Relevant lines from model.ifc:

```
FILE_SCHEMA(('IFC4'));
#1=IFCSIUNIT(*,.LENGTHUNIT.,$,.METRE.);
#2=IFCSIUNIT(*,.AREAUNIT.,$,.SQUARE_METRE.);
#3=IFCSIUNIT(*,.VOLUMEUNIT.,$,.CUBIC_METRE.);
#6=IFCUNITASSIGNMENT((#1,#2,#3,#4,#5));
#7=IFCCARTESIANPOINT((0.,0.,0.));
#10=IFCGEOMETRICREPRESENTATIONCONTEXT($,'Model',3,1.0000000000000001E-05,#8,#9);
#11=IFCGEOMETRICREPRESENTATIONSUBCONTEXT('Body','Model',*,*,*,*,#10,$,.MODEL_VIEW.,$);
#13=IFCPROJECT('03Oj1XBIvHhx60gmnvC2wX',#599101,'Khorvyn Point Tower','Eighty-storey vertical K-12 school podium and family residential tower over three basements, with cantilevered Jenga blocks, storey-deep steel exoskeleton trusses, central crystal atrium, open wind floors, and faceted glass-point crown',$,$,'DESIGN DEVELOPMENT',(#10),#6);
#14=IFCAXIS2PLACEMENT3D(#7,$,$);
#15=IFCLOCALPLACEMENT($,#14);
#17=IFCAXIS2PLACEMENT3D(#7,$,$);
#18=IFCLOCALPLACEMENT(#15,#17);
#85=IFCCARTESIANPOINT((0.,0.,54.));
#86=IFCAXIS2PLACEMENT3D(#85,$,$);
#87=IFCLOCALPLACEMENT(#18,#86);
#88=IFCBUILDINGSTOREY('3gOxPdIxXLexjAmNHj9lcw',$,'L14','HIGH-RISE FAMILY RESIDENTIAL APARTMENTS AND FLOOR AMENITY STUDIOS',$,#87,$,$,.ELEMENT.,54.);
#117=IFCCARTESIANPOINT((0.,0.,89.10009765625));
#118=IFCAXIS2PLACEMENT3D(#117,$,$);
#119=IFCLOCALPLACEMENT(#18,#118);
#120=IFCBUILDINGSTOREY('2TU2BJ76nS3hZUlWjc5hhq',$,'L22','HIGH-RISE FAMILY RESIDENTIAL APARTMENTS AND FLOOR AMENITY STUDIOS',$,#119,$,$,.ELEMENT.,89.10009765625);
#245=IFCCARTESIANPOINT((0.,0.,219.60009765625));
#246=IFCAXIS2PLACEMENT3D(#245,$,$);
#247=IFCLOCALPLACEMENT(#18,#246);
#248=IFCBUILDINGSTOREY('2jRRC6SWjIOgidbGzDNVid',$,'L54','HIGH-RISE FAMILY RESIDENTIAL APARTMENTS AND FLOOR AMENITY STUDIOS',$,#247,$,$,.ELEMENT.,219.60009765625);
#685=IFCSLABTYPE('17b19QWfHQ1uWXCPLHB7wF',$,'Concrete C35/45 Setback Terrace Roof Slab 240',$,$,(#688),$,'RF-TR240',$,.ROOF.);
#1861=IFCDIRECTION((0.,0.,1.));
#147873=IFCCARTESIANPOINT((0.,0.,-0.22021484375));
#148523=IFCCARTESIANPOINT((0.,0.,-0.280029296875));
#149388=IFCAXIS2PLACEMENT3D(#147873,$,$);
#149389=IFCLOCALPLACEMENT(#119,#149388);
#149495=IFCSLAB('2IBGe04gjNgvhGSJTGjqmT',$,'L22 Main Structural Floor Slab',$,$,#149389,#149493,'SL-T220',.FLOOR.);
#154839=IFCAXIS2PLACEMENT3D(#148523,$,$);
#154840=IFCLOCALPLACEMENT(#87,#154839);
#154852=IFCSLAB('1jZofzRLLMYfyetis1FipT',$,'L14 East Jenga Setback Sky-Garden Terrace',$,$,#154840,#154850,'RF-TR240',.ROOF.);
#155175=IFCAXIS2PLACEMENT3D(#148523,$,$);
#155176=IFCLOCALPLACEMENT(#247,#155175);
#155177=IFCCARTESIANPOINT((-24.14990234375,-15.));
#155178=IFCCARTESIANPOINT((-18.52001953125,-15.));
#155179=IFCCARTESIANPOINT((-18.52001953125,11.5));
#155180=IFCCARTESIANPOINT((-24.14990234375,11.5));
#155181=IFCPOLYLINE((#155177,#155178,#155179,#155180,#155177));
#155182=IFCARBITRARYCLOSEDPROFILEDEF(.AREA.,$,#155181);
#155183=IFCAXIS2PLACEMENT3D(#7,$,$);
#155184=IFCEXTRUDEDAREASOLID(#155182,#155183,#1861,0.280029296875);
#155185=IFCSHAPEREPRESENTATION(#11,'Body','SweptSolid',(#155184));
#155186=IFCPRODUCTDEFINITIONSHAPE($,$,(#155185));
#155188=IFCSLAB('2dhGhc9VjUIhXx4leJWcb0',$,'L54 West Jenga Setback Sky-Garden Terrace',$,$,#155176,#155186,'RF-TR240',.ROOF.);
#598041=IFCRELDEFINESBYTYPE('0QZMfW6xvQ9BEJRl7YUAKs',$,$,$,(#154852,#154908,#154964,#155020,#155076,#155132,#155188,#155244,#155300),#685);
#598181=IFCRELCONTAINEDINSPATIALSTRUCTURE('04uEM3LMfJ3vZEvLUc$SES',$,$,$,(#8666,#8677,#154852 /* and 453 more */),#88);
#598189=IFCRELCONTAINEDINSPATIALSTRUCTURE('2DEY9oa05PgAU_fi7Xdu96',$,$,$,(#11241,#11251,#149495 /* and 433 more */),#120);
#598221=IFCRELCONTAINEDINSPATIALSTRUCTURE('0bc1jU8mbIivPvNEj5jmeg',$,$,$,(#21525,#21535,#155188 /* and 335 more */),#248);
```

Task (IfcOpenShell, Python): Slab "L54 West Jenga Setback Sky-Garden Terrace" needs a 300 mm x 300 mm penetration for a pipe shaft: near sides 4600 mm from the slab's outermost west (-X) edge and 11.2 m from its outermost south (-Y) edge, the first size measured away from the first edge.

```python
import numpy as np
import ifcopenshell
import ifcopenshell.api.feature
import ifcopenshell.api.geometry
import ifcopenshell.api.root
import ifcopenshell.geom
import ifcopenshell.util.placement
import ifcopenshell.util.representation
import ifcopenshell.util.shape
import ifcopenshell.util.unit

model = ifcopenshell.open("model.ifc")
unit_scale = ifcopenshell.util.unit.calculate_unit_scale(model)
settings = ifcopenshell.geom.settings()


def volume(element):
    """Net volume in cubic metres, openings subtracted."""
    shape = ifcopenshell.geom.create_shape(settings, element)
    return ifcopenshell.util.shape.get_volume(shape.geometry)


slab = model.by_guid("2dhGhc9VjUIhXx4leJWcb0")
before = volume(slab)

# Extent in the slab's own axes, in metres. The edges named are its -X and -Y sides.
slab_shape = ifcopenshell.geom.create_shape(settings, slab)
vertices = ifcopenshell.util.shape.get_vertices(slab_shape.geometry)
x_min, y_min, bottom = vertices.min(axis=0)
top = vertices[:, 2].max()

opening = ifcopenshell.api.root.create_entity(model, ifc_class="IfcOpeningElement", name="Pipe shaft opening", predefined_type="OPENING")
context = ifcopenshell.util.representation.get_context(model, "Model", "Body", "MODEL_VIEW")
width, depth = 0.3, 0.3
outline = [(0.0, 0.0), (width, 0.0), (width, depth), (0.0, depth), (0.0, 0.0)]
# Overshoot both faces by 50 mm so the cut is clean.
shape = ifcopenshell.api.geometry.add_slab_representation(
    model, context=context, depth=top - bottom + 0.1, polyline=outline
)
ifcopenshell.api.geometry.assign_representation(model, product=opening, representation=shape)

matrix = ifcopenshell.util.placement.get_local_placement(slab.ObjectPlacement)
matrix[:, 3] = matrix @ np.append(np.array([x_min + 4.6, y_min + 11.2, bottom - 0.05]) / unit_scale, 1.0)
ifcopenshell.api.geometry.edit_object_placement(model, product=opening, matrix=matrix, is_si=False)
ifcopenshell.api.feature.add_feature(model, feature=opening, element=slab)

after = volume(slab)

print(f"slab volume {before:.3f} -> {after:.3f} m3")

model.write("model-out.ifc")
```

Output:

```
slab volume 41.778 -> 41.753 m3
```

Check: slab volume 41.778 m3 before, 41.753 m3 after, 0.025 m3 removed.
